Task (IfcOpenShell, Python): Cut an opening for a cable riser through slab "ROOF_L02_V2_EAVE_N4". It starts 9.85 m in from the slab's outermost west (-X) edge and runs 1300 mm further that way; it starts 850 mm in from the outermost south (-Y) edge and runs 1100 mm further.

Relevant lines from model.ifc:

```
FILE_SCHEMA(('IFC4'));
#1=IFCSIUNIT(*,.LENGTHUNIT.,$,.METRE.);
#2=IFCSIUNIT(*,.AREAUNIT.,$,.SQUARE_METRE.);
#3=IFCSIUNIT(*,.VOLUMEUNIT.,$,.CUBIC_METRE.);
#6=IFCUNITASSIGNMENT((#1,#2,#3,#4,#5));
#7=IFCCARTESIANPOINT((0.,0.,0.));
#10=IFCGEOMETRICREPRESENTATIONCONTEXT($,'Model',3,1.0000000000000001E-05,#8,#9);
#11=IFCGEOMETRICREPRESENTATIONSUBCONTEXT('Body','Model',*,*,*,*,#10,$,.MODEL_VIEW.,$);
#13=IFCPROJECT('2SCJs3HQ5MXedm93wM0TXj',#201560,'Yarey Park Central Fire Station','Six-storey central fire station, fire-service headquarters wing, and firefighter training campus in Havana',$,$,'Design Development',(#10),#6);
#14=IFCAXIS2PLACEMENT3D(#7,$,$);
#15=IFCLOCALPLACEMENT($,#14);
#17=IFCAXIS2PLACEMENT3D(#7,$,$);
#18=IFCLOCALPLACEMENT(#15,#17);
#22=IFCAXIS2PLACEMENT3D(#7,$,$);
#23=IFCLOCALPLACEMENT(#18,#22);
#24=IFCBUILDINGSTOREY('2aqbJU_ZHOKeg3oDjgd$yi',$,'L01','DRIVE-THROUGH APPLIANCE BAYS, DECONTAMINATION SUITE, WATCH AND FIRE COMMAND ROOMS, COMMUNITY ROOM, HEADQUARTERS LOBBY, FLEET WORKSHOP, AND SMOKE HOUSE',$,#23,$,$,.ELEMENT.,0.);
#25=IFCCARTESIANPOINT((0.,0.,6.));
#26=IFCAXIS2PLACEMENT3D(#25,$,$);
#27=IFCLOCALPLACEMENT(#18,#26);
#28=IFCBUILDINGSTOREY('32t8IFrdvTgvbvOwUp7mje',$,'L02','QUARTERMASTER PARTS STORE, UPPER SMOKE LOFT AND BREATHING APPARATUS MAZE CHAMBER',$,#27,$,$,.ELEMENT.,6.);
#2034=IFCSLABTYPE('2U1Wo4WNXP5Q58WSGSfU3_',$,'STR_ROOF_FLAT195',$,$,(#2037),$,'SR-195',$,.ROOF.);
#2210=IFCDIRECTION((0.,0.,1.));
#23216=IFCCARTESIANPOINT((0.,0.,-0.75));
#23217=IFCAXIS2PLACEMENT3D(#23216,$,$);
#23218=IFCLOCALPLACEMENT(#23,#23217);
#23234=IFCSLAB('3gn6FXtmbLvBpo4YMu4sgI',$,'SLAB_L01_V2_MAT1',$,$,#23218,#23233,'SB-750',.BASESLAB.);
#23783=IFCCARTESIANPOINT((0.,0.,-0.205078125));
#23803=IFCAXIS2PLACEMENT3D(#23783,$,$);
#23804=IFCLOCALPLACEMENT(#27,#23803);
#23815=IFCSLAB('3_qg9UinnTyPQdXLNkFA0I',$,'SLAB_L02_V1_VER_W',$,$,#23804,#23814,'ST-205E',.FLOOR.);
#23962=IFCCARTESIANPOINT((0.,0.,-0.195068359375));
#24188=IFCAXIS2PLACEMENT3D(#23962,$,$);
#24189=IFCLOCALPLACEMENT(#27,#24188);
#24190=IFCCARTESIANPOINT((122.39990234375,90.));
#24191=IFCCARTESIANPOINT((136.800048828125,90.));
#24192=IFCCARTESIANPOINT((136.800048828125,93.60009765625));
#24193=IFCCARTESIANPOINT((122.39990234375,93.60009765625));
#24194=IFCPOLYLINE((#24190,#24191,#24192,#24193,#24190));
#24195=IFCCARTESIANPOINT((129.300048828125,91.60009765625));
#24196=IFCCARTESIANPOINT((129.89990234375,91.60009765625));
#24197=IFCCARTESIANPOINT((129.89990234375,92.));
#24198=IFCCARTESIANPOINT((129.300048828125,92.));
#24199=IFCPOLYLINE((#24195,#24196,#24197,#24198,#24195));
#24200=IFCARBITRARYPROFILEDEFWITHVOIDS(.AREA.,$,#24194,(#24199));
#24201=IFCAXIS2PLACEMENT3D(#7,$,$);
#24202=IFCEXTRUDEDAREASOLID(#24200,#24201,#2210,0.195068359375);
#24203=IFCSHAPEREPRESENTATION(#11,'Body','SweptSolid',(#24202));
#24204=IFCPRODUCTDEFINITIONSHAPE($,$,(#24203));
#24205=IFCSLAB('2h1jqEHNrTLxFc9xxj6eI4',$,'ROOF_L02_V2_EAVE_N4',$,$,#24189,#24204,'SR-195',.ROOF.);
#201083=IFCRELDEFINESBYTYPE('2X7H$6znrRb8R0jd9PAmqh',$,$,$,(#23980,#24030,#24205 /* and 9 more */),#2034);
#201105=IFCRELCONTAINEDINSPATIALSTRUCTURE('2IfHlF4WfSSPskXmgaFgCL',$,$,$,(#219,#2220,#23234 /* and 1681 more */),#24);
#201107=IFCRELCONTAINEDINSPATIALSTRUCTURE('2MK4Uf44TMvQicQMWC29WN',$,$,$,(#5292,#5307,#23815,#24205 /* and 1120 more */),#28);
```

```python
import numpy as np
import ifcopenshell
import ifcopenshell.api.feature
import ifcopenshell.api.geometry
import ifcopenshell.api.root
import ifcopenshell.geom
import ifcopenshell.util.placement
import ifcopenshell.util.representation
import ifcopenshell.util.shape
import ifcopenshell.util.unit

model = ifcopenshell.open("model.ifc")
unit_scale = ifcopenshell.util.unit.calculate_unit_scale(model)
settings = ifcopenshell.geom.settings()


def volume(element):
    """Net volume in cubic metres, openings subtracted."""
    shape = ifcopenshell.geom.create_shape(settings, element)
    return ifcopenshell.util.shape.get_volume(shape.geometry)


slab = model.by_guid("2h1jqEHNrTLxFc9xxj6eI4")
before = volume(slab)

# Extent in the slab's own axes, in metres. The edges named are its -X and -Y sides.
slab_shape = ifcopenshell.geom.create_shape(settings, slab)
vertices = ifcopenshell.util.shape.get_vertices(slab_shape.geometry)
x_min, y_min, bottom = vertices.min(axis=0)
top = vertices[:, 2].max()

opening = ifcopenshell.api.root.create_entity(model, ifc_class="IfcOpeningElement", name="Cable riser opening", predefined_type="OPENING")
context = ifcopenshell.util.representation.get_context(model, "Model", "Body", "MODEL_VIEW")
width, depth = 1.3, 1.1
outline = [(0.0, 0.0), (width, 0.0), (width, depth), (0.0, depth), (0.0, 0.0)]
# Overshoot both faces by 50 mm so the cut is clean.
shape = ifcopenshell.api.geometry.add_slab_representation(
    model, context=context, depth=top - bottom + 0.1, polyline=outline
)
ifcopenshell.api.geometry.assign_representation(model, product=opening, representation=shape)

matrix = ifcopenshell.util.placement.get_local_placement(slab.ObjectPlacement)
matrix[:, 3] = matrix @ np.append(np.array([x_min + 9.85, y_min + 0.85, bottom - 0.05]) / unit_scale, 1.0)
ifcopenshell.api.geometry.edit_object_placement(model, product=opening, matrix=matrix, is_si=False)
ifcopenshell.api.feature.add_feature(model, feature=opening, element=slab)

after = volume(slab)

print(f"slab volume {before:.3f} -> {after:.3f} m3")

model.write("model_updated.ifc")
```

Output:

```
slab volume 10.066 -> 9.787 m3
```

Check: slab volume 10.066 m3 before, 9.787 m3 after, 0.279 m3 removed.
